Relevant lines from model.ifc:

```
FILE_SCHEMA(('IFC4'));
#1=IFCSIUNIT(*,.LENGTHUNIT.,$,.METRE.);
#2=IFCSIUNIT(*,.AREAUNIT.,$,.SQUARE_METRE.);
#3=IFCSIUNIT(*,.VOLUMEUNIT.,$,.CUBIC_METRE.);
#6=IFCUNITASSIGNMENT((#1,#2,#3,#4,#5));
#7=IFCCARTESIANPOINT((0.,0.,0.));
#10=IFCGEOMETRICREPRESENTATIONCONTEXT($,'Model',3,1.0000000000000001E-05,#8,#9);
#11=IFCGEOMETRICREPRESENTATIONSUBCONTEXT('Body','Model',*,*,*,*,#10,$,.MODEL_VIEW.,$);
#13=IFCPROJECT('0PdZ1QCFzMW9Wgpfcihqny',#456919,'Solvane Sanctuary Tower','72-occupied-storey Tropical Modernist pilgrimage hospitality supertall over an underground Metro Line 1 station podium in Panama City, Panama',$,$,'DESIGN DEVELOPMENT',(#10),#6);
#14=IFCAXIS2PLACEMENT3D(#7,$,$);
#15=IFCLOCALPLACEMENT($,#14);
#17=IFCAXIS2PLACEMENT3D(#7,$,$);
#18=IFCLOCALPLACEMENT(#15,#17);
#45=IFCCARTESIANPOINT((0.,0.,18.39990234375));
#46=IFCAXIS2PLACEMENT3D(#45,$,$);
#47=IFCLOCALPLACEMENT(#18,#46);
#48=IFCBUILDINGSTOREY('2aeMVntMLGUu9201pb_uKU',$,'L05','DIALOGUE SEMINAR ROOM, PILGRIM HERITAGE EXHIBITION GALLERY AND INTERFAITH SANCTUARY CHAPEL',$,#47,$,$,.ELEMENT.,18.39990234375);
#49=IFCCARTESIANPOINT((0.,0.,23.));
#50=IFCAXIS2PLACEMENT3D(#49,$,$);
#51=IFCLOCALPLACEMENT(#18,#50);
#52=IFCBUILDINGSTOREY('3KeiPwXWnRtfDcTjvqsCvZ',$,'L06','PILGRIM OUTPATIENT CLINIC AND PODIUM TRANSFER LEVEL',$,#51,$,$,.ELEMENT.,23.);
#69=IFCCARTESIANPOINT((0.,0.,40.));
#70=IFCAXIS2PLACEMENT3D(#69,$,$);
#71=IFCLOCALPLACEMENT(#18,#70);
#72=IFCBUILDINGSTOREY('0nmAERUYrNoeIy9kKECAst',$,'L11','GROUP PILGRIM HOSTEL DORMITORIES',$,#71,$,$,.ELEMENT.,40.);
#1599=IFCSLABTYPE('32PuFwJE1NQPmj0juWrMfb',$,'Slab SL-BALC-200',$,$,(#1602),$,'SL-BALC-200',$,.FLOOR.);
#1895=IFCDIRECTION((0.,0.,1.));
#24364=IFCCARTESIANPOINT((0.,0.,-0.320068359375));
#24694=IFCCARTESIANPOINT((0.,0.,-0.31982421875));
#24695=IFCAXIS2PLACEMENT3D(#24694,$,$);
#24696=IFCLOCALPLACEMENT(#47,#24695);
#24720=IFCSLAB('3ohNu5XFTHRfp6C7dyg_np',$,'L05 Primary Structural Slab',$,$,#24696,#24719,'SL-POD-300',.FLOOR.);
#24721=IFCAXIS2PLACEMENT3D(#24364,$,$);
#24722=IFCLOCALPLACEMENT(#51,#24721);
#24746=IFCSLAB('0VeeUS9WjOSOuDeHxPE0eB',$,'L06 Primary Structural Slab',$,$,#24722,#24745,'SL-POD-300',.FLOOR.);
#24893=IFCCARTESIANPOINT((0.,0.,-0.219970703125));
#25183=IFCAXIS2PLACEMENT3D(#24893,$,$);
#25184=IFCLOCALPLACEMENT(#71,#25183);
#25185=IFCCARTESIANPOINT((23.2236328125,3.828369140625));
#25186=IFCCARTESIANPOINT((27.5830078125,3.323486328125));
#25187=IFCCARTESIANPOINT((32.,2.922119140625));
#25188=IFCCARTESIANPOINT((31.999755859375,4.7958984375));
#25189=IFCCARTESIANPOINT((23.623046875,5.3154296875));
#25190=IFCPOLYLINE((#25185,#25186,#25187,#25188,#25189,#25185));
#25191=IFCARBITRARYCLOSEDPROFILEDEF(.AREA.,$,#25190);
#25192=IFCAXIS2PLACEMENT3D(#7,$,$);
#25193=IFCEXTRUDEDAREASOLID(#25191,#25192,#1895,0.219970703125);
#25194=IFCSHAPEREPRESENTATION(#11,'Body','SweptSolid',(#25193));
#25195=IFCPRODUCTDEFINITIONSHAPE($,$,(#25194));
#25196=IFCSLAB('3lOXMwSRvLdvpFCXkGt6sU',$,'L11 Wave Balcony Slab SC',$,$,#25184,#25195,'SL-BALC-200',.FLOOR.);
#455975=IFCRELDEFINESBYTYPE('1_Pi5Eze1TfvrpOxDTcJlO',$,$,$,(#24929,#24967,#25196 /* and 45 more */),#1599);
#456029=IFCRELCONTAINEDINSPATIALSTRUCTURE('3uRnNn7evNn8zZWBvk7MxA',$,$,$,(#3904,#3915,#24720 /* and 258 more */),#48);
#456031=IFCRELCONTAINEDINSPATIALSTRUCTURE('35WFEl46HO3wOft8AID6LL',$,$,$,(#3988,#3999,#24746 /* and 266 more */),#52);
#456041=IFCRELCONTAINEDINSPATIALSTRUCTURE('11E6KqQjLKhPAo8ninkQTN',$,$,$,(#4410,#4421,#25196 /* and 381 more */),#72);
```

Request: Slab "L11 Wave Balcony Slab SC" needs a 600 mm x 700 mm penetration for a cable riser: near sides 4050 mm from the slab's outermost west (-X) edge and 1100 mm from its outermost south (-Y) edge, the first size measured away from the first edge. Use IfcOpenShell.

```python
import numpy as np
import ifcopenshell
import ifcopenshell.api.feature
import ifcopenshell.api.geometry
import ifcopenshell.api.root
import ifcopenshell.geom
import ifcopenshell.util.placement
import ifcopenshell.util.representation
import ifcopenshell.util.shape
import ifcopenshell.util.unit

model = ifcopenshell.open("model.ifc")
unit_scale = ifcopenshell.util.unit.calculate_unit_scale(model)
settings = ifcopenshell.geom.settings()


def volume(element):
    """Net volume in cubic metres, openings subtracted."""
    shape = ifcopenshell.geom.create_shape(settings, element)
    return ifcopenshell.util.shape.get_volume(shape.geometry)


slab = model.by_guid("3lOXMwSRvLdvpFCXkGt6sU")
before = volume(slab)

# Extent in the slab's own axes, in metres. The edges named are its -X and -Y sides.
slab_shape = ifcopenshell.geom.create_shape(settings, slab)
vertices = ifcopenshell.util.shape.get_vertices(slab_shape.geometry)
x_min, y_min, bottom = vertices.min(axis=0)
top = vertices[:, 2].max()

opening = ifcopenshell.api.root.create_entity(model, ifc_class="IfcOpeningElement", name="Cable riser opening", predefined_type="OPENING")
context = ifcopenshell.util.representation.get_context(model, "Model", "Body", "MODEL_VIEW")
width, depth = 0.6, 0.7
outline = [(0.0, 0.0), (width, 0.0), (width, depth), (0.0, depth), (0.0, 0.0)]
# Overshoot both faces by 50 mm so the cut is clean.
shape = ifcopenshell.api.geometry.add_slab_representation(
    model, context=context, depth=top - bottom + 0.1, polyline=outline
)
ifcopenshell.api.geometry.assign_representation(model, product=opening, representation=shape)

matrix = ifcopenshell.util.placement.get_local_placement(slab.ObjectPlacement)
matrix[:, 3] = matrix @ np.append(np.array([x_min + 4.05, y_min + 1.1, bottom - 0.05]) / unit_scale, 1.0)
ifcopenshell.api.geometry.edit_object_placement(model, product=opening, matrix=matrix, is_si=False)
ifcopenshell.api.feature.add_feature(model, feature=opening, element=slab)

after = volume(slab)

print(f"slab volume {before:.3f} -> {after:.3f} m3")

model.write("model_v2.ifc")
```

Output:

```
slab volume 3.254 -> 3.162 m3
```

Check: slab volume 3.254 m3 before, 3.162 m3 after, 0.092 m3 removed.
